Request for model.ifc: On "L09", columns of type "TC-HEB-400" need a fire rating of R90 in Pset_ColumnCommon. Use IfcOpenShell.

First a look at what the model holds.

```python
import ifcopenshell
import ifcopenshell.util.element

model = ifcopenshell.open("model.ifc")
print(model.schema)
storey = next(s for s in model.by_type("IfcBuildingStorey") if s.Name == "L09")
columns = [e for e in ifcopenshell.util.element.get_decomposition(storey) if e.is_a("IfcColumn")]
seen = {}
for e in columns:
    element_type = ifcopenshell.util.element.get_type(e)
    key = (element_type.Name if element_type != e and element_type else None, ifcopenshell.util.element.get_pset(e, "Pset_ColumnCommon", "FireRating"))
    seen[key] = seen.get(key, 0) + 1
for (name, value), count in sorted(seen.items(), key=str):
    print(count, "x", name, "|", value)
```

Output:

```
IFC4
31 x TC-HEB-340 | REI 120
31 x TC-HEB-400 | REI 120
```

```python
import ifcopenshell
import ifcopenshell.api.pset
import ifcopenshell.util.element

model = ifcopenshell.open("model.ifc")

storey = next(s for s in model.by_type("IfcBuildingStorey") if s.Name == "L09")
columns = [e for e in ifcopenshell.util.element.get_decomposition(storey) if e.is_a("IfcColumn")]

count = 0
for e in columns:
    element_type = ifcopenshell.util.element.get_type(e)
    if element_type in (None, e) or element_type.Name != "TC-HEB-400":
        continue
    # add_pset returns the element's existing set when there is one.
    pset = ifcopenshell.api.pset.add_pset(model, product=e, name="Pset_ColumnCommon")
    ifcopenshell.api.pset.edit_pset(model, pset=pset, properties={"FireRating": "R90"})
    count += 1

print(count, "columns updated")

model.write("model-out.ifc")
```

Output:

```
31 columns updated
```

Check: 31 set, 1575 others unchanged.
